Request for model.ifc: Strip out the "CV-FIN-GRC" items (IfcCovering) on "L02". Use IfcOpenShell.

First a look at what the model holds.

```python
import ifcopenshell
import ifcopenshell.util.element

model = ifcopenshell.open("model.ifc")
print(model.schema)
storey = next(s for s in model.by_type("IfcBuildingStorey") if s.Name == "L02")
coverings = [e for e in ifcopenshell.util.element.get_decomposition(storey) if e.is_a("IfcCovering")]
seen = {}
for e in coverings:
    element_type = ifcopenshell.util.element.get_type(e)
    name = element_type.Name if element_type not in (None, e) else None
    seen[name] = seen.get(name, 0) + 1
for name, count in sorted(seen.items(), key=str):
    print(count, "x", name)
```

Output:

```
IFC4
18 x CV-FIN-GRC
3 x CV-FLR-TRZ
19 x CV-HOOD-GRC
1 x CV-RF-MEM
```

```python
import ifcopenshell
import ifcopenshell.api.root
import ifcopenshell.util.element

model = ifcopenshell.open("model.ifc")

storey = next(s for s in model.by_type("IfcBuildingStorey") if s.Name == "L02")
coverings = [e for e in ifcopenshell.util.element.get_decomposition(storey) if e.is_a("IfcCovering")]
targets = [e for e in coverings if (t := ifcopenshell.util.element.get_type(e)) not in (None, e) and t.Name == "CV-FIN-GRC"]

for e in targets:
    ifcopenshell.api.root.remove_product(model, product=e)
print(len(targets), "removed")

model.write("model_updated.ifc")
```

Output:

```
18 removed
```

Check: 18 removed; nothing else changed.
